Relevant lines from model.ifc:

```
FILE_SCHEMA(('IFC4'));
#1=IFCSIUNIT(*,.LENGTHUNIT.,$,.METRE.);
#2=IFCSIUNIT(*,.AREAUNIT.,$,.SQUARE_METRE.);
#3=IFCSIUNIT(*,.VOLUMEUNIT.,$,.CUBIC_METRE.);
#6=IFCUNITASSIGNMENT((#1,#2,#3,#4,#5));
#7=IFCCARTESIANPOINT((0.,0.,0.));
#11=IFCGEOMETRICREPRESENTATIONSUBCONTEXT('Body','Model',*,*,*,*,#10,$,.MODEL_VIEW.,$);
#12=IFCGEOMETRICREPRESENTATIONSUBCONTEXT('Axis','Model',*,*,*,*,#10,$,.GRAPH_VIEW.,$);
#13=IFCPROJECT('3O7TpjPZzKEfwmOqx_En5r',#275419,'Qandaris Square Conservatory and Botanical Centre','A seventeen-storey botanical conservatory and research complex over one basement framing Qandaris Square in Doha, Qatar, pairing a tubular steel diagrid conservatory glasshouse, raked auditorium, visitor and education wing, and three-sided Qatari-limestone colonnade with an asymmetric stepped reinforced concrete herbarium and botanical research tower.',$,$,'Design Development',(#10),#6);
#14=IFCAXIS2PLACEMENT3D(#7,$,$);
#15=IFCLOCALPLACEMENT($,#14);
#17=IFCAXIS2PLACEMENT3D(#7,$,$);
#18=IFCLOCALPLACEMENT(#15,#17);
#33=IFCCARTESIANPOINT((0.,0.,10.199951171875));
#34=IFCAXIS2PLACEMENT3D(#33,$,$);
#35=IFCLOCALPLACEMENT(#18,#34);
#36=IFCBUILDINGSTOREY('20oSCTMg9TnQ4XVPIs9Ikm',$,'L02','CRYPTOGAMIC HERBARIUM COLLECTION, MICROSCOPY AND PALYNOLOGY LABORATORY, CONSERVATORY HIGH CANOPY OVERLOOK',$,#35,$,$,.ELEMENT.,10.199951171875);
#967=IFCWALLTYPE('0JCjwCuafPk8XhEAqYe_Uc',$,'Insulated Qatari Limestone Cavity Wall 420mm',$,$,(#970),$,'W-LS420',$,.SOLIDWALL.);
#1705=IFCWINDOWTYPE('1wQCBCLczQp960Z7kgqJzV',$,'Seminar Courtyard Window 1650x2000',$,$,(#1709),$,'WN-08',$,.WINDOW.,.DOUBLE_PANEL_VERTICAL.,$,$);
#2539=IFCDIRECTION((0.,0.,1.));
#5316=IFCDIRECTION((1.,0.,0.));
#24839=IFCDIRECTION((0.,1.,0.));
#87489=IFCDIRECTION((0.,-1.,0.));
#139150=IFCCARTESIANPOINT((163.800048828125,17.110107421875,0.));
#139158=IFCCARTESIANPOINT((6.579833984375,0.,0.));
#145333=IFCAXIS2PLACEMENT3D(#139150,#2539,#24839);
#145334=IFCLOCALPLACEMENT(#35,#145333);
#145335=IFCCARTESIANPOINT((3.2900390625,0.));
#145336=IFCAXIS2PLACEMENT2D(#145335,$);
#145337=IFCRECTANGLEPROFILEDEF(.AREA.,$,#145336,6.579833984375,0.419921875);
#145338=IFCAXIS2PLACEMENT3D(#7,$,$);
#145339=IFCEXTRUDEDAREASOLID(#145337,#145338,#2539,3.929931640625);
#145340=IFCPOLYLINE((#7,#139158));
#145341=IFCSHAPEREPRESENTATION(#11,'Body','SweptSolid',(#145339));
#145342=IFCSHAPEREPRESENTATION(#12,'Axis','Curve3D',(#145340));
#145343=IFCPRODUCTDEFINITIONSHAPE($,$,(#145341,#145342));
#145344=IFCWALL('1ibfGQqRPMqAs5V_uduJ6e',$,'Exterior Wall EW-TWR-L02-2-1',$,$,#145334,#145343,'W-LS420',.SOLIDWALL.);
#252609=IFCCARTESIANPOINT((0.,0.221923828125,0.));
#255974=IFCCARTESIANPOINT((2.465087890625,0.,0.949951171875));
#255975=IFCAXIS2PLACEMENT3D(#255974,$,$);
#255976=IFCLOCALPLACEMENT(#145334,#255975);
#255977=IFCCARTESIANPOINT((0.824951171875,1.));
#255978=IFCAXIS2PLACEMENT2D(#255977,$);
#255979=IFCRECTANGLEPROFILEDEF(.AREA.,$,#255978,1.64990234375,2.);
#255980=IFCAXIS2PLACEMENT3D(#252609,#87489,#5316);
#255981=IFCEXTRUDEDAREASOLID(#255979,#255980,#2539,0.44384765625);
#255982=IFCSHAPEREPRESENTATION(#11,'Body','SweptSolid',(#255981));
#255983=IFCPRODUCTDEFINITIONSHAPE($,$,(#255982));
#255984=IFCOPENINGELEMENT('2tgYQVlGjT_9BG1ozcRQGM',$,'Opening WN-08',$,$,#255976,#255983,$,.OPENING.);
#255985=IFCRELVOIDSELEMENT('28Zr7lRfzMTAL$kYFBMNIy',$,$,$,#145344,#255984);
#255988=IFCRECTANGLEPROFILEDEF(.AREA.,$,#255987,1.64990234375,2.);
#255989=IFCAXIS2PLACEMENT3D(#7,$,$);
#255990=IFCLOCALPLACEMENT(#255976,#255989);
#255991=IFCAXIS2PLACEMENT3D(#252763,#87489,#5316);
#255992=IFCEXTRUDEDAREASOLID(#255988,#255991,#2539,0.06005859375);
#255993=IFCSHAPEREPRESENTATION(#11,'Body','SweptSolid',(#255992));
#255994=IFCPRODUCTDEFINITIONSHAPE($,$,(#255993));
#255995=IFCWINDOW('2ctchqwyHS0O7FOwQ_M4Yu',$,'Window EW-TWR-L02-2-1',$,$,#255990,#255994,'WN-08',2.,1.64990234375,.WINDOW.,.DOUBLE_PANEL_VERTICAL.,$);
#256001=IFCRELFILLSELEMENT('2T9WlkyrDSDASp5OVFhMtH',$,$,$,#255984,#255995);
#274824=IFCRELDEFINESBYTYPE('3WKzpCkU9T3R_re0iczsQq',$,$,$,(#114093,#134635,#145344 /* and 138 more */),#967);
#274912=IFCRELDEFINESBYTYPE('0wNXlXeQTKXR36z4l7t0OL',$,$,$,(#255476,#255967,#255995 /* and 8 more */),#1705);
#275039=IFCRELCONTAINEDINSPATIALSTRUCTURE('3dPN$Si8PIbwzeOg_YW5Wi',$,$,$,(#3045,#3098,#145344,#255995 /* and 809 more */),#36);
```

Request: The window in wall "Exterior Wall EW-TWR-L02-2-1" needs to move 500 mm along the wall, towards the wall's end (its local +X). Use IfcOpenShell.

```python
import ifcopenshell
import ifcopenshell.api.geometry
import ifcopenshell.util.placement
import ifcopenshell.util.unit

model = ifcopenshell.open("model.ifc")
unit_scale = ifcopenshell.util.unit.calculate_unit_scale(model)

window = model.by_guid("2ctchqwyHS0O7FOwQ_M4Yu")
opening = window.FillsVoids[0].RelatingOpeningElement
wall = opening.VoidsElements[0].RelatingBuildingElement

wall_matrix = ifcopenshell.util.placement.get_local_placement(wall.ObjectPlacement)
shift = wall_matrix[:3, 0] * 0.5 / unit_scale
before = ifcopenshell.util.placement.get_local_placement(window.ObjectPlacement)[:3, 3].copy()

# The window is placed relative to its opening, so it follows when the opening moves.
matrix = ifcopenshell.util.placement.get_local_placement(opening.ObjectPlacement)
matrix[:3, 3] += shift
ifcopenshell.api.geometry.edit_object_placement(
    model, product=opening, matrix=matrix, is_si=False, should_transform_children=True
)

after = ifcopenshell.util.placement.get_local_placement(window.ObjectPlacement)[:3, 3]
print("window moved by", (after - before).round(3) + 0.0)

model.write("model_v2.ifc")
```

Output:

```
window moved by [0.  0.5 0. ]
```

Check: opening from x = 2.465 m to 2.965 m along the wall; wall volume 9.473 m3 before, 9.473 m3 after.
